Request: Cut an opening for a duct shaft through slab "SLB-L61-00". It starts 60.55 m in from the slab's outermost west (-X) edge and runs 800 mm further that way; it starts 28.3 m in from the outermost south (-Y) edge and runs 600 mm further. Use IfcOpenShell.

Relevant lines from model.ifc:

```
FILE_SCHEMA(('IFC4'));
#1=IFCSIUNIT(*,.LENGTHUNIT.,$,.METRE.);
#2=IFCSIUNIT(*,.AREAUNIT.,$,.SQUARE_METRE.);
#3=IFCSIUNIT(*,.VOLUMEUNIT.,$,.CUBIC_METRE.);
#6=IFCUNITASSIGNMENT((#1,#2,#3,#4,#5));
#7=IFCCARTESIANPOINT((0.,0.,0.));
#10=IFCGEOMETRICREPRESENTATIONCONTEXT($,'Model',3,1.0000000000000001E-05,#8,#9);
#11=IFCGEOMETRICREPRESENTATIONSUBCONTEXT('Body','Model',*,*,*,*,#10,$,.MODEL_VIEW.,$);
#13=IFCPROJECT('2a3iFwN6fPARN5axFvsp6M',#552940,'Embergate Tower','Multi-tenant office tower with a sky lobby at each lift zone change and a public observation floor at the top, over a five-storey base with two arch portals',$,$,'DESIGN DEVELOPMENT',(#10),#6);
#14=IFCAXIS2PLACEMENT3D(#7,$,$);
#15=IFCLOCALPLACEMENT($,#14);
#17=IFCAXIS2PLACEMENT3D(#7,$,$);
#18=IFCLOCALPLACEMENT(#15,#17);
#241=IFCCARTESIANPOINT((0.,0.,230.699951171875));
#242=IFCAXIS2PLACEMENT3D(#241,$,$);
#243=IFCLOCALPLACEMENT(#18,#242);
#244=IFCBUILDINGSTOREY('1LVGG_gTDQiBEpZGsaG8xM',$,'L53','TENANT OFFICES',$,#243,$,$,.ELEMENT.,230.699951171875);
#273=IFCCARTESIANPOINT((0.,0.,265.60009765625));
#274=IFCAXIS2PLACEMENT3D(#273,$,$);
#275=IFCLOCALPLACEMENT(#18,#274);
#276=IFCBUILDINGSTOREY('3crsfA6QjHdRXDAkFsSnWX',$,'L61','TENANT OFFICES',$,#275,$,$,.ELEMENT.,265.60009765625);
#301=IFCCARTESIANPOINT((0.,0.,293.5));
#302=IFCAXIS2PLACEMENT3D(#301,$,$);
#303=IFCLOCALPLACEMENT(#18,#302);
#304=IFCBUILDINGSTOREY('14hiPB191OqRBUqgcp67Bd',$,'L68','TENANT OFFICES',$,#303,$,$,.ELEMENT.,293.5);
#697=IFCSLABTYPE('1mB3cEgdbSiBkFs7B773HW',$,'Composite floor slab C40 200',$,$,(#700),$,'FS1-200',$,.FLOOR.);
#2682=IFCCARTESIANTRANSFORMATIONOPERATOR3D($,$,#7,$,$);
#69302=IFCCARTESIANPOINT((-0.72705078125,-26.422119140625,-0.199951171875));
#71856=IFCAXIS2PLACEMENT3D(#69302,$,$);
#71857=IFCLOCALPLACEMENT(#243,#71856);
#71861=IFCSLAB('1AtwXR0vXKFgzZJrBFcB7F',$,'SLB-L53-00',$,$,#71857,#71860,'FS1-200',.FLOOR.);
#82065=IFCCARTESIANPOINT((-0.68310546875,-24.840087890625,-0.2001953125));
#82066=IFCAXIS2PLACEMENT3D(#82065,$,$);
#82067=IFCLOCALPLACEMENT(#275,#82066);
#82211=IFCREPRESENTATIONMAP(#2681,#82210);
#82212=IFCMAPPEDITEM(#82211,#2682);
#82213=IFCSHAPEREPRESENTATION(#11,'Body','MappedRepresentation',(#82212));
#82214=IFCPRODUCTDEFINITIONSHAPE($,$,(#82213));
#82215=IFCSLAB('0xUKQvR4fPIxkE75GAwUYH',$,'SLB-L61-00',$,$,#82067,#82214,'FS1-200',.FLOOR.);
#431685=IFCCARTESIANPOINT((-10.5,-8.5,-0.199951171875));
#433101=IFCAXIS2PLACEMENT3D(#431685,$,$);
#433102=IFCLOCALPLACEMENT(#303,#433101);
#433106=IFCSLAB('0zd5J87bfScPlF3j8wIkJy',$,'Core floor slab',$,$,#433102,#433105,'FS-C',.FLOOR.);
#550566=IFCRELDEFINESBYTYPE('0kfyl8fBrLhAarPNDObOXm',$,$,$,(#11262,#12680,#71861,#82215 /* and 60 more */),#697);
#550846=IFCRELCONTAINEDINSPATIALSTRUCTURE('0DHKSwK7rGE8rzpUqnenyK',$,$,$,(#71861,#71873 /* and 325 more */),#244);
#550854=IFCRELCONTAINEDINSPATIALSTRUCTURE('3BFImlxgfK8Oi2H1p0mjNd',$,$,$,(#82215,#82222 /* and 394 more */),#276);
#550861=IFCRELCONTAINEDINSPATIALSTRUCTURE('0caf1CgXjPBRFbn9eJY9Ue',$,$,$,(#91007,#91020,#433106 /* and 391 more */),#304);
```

```python
import numpy as np
import ifcopenshell
import ifcopenshell.api.feature
import ifcopenshell.api.geometry
import ifcopenshell.api.root
import ifcopenshell.geom
import ifcopenshell.util.placement
import ifcopenshell.util.representation
import ifcopenshell.util.shape
import ifcopenshell.util.unit

model = ifcopenshell.open("model.ifc")
unit_scale = ifcopenshell.util.unit.calculate_unit_scale(model)
settings = ifcopenshell.geom.settings()


def volume(element):
    """Net volume in cubic metres, openings subtracted."""
    shape = ifcopenshell.geom.create_shape(settings, element)
    return ifcopenshell.util.shape.get_volume(shape.geometry)


slab = model.by_guid("0xUKQvR4fPIxkE75GAwUYH")
before = volume(slab)

# Extent in the slab's own axes, in metres. The edges named are its -X and -Y sides.
slab_shape = ifcopenshell.geom.create_shape(settings, slab)
vertices = ifcopenshell.util.shape.get_vertices(slab_shape.geometry)
x_min, y_min, bottom = vertices.min(axis=0)
top = vertices[:, 2].max()

opening = ifcopenshell.api.root.create_entity(model, ifc_class="IfcOpeningElement", name="Duct shaft opening", predefined_type="OPENING")
context = ifcopenshell.util.representation.get_context(model, "Model", "Body", "MODEL_VIEW")
width, depth = 0.8, 0.6
outline = [(0.0, 0.0), (width, 0.0), (width, depth), (0.0, depth), (0.0, 0.0)]
# Overshoot both faces by 50 mm so the cut is clean.
shape = ifcopenshell.api.geometry.add_slab_representation(
    model, context=context, depth=top - bottom + 0.1, polyline=outline
)
ifcopenshell.api.geometry.assign_representation(model, product=opening, representation=shape)

matrix = ifcopenshell.util.placement.get_local_placement(slab.ObjectPlacement)
matrix[:, 3] = matrix @ np.append(np.array([x_min + 60.55, y_min + 28.3, bottom - 0.05]) / unit_scale, 1.0)
ifcopenshell.api.geometry.edit_object_placement(model, product=opening, matrix=matrix, is_si=False)
ifcopenshell.api.feature.add_feature(model, feature=opening, element=slab)

after = volume(slab)

print(f"slab volume {before:.3f} -> {after:.3f} m3")

model.write("model_updated.ifc")
```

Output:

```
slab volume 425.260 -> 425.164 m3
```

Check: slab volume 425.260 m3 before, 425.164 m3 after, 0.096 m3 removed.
